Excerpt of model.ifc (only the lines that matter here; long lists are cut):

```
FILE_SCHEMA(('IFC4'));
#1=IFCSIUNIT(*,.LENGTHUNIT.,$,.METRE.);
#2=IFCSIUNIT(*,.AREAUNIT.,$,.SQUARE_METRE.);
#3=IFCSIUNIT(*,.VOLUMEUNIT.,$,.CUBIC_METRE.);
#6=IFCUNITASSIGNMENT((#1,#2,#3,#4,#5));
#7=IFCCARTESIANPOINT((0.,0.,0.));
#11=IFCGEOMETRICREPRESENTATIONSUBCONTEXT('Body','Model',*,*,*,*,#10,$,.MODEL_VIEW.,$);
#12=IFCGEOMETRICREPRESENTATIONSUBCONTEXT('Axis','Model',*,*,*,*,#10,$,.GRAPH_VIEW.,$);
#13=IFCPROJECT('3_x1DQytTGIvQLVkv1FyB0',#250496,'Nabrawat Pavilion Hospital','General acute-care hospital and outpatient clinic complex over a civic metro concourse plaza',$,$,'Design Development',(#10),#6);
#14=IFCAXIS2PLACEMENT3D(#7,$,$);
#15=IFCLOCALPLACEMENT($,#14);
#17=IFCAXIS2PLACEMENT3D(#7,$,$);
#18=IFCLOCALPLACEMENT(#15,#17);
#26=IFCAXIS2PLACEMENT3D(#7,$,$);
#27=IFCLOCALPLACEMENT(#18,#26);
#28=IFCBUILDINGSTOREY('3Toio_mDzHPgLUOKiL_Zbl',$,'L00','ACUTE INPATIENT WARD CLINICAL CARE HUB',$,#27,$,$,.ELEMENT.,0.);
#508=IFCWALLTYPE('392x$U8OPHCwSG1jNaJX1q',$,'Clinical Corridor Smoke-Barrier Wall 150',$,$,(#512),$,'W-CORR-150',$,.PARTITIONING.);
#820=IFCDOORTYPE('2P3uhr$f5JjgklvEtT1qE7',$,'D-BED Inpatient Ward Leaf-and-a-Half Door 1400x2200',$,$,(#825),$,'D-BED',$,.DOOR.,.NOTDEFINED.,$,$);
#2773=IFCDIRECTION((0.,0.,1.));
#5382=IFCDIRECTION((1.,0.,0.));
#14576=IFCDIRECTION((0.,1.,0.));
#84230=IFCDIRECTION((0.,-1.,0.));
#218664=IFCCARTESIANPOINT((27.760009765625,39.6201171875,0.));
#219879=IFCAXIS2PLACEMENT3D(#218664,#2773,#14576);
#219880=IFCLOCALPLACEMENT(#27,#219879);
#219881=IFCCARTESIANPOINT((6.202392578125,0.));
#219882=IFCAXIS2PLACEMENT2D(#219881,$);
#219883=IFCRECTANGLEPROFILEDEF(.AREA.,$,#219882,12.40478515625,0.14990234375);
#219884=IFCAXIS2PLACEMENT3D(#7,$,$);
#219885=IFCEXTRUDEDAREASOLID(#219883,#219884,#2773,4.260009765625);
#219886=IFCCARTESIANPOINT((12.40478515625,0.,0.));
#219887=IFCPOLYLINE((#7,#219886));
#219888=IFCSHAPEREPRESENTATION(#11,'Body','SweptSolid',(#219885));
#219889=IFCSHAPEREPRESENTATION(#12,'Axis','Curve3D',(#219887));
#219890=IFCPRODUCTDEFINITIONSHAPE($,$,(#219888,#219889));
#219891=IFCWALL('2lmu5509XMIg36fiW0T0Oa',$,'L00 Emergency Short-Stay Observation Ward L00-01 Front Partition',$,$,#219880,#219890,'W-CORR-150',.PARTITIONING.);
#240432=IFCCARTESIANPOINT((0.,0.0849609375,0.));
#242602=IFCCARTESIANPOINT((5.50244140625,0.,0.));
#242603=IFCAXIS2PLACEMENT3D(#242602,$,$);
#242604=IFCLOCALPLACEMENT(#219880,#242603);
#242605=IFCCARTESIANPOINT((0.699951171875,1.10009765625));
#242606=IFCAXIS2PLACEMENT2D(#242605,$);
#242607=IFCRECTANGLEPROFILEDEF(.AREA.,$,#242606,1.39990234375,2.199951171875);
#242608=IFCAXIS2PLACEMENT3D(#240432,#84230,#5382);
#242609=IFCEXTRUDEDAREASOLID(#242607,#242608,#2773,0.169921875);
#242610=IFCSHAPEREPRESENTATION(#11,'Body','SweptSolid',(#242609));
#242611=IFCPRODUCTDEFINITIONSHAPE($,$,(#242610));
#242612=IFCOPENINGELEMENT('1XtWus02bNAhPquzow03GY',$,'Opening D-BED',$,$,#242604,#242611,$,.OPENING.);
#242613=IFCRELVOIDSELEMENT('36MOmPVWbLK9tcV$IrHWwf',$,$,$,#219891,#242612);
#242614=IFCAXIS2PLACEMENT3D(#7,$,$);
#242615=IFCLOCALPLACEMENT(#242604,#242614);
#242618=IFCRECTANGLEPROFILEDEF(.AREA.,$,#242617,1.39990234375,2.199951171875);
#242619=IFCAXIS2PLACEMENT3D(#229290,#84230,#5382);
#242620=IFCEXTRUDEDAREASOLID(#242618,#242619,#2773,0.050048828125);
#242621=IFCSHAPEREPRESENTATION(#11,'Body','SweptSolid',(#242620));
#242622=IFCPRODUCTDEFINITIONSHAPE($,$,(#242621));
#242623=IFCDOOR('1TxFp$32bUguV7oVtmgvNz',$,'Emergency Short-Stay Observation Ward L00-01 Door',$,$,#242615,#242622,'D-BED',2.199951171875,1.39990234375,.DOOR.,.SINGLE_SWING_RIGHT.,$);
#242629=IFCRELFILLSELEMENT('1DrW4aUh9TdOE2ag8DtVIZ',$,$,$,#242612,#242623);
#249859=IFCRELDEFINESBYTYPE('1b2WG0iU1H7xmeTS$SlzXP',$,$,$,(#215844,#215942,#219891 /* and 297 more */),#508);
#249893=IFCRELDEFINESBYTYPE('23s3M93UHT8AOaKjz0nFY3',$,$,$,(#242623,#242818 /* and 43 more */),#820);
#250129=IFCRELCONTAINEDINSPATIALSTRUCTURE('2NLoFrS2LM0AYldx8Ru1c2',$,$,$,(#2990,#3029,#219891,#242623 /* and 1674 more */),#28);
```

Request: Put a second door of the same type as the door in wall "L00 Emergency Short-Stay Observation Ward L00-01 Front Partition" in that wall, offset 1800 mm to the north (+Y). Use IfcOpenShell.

```python
import ifcopenshell
import ifcopenshell.api.feature
import ifcopenshell.api.geometry
import ifcopenshell.api.root
import ifcopenshell.geom
import ifcopenshell.util.element
import ifcopenshell.util.placement
import ifcopenshell.util.shape

model = ifcopenshell.open("model.ifc")
settings = ifcopenshell.geom.settings()


def volume(element):
    """Net volume in cubic metres, openings subtracted."""
    shape = ifcopenshell.geom.create_shape(settings, element)
    return ifcopenshell.util.shape.get_volume(shape.geometry)


door = model.by_guid("1TxFp$32bUguV7oVtmgvNz")
opening = door.FillsVoids[0].RelatingOpeningElement
wall = opening.VoidsElements[0].RelatingBuildingElement
before = volume(wall)
shift = ifcopenshell.util.placement.get_local_placement(wall.ObjectPlacement)[:3, 0] * 1.8

# copy_class copies the void relationship, type, container and properties, but no geometry.
new_opening = ifcopenshell.api.root.copy_class(model, product=opening)
new_opening.Representation = ifcopenshell.util.element.copy_deep(
    model, opening.Representation, exclude=["IfcGeometricRepresentationContext", "IfcRepresentationMap"]
)
new_door = ifcopenshell.api.root.copy_class(model, product=door)
new_door.Representation = ifcopenshell.util.element.copy_deep(
    model, door.Representation, exclude=["IfcGeometricRepresentationContext", "IfcRepresentationMap"]
)
new_door.Tag = None
ifcopenshell.api.feature.add_filling(model, opening=new_opening, element=new_door)

for old, new in ((opening, new_opening), (door, new_door)):
    matrix = ifcopenshell.util.placement.get_local_placement(old.ObjectPlacement)
    matrix[:3, 3] += shift
    ifcopenshell.api.geometry.edit_object_placement(model, product=new, matrix=matrix, is_si=False)

after = volume(wall)

print(f"wall volume {before:.3f} -> {after:.3f} m3")

model.write("model_rev.ifc")
```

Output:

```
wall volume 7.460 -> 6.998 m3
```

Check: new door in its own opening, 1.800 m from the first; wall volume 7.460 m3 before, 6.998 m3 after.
